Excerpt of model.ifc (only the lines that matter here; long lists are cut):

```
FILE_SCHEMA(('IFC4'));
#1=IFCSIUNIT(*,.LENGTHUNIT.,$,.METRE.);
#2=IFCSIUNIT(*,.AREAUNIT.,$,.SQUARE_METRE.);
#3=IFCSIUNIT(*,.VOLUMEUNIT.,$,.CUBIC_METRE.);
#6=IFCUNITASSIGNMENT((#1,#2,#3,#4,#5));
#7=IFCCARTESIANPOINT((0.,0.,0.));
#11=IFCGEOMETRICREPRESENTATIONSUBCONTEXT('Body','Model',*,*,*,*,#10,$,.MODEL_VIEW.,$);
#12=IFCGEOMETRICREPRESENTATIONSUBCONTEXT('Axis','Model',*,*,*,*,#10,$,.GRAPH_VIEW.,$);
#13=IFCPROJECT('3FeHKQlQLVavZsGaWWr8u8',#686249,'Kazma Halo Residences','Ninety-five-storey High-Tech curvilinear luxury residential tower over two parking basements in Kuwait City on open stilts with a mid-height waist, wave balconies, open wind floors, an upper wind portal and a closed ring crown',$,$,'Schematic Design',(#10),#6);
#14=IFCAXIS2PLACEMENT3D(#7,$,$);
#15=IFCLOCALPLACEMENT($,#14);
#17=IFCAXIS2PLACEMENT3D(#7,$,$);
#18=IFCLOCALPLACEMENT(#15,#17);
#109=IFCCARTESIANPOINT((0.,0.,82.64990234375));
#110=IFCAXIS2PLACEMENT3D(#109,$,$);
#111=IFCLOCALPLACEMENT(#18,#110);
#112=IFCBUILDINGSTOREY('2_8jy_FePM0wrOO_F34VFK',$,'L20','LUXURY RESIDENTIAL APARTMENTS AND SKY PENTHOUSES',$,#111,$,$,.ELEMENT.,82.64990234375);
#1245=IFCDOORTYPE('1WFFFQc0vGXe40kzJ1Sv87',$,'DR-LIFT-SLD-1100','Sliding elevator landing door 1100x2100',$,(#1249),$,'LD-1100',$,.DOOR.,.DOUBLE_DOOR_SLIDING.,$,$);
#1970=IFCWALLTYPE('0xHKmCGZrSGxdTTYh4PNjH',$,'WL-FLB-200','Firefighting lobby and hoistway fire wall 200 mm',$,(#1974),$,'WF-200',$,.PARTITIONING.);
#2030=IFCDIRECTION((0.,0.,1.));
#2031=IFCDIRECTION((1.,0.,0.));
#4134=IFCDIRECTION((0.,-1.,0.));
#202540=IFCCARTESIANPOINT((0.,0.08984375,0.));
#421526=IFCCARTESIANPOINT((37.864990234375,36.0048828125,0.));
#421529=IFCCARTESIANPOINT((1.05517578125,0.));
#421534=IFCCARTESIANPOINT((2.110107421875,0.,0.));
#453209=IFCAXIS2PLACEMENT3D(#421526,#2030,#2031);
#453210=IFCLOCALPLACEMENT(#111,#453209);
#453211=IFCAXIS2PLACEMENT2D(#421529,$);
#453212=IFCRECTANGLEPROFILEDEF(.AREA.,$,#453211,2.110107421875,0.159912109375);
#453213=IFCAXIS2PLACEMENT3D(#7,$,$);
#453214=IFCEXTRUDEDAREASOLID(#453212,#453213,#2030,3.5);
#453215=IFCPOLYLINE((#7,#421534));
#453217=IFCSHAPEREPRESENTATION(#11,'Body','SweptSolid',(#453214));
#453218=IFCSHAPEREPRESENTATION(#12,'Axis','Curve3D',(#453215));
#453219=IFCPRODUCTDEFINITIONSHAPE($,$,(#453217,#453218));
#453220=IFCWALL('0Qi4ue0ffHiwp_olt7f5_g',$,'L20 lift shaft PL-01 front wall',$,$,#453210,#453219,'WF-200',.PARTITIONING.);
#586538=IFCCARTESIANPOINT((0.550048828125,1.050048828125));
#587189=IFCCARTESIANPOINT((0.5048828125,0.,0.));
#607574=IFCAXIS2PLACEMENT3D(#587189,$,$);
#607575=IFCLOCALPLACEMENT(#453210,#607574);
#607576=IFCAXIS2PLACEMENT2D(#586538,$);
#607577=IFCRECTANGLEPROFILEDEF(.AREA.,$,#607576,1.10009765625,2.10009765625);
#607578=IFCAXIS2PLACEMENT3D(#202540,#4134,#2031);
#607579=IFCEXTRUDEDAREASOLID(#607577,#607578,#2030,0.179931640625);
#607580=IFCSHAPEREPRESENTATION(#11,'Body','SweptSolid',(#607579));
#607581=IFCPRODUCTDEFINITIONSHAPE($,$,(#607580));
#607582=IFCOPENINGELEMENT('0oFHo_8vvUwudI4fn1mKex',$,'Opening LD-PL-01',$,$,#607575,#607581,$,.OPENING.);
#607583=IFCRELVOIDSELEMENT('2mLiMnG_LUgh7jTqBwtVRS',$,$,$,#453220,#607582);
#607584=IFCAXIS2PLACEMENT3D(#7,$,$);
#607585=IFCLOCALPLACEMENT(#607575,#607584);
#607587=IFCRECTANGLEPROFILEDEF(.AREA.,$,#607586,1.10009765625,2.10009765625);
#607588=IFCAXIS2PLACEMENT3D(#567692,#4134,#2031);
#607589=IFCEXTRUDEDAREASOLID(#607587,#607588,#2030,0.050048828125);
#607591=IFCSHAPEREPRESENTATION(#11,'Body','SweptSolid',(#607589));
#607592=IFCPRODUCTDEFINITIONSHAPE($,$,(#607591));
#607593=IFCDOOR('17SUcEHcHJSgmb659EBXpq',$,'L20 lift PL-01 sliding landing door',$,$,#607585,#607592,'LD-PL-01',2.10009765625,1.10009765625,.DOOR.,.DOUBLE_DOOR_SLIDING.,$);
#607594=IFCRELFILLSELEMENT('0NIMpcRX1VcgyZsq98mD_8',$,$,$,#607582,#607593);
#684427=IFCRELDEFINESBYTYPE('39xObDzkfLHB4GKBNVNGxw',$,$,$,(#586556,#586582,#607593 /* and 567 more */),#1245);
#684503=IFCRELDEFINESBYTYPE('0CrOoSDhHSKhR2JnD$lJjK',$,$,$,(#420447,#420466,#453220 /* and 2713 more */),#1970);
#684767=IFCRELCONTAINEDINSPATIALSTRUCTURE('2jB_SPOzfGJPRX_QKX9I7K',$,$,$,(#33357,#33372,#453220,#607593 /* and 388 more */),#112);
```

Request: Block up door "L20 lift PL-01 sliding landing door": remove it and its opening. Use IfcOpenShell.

```python
import ifcopenshell
import ifcopenshell.api.feature
import ifcopenshell.api.root
import ifcopenshell.geom
import ifcopenshell.util.shape

model = ifcopenshell.open("model.ifc")
settings = ifcopenshell.geom.settings()


def volume(element):
    """Net volume in cubic metres, openings subtracted."""
    shape = ifcopenshell.geom.create_shape(settings, element)
    return ifcopenshell.util.shape.get_volume(shape.geometry)


door = model.by_guid("17SUcEHcHJSgmb659EBXpq")
opening = door.FillsVoids[0].RelatingOpeningElement
wall = opening.VoidsElements[0].RelatingBuildingElement
before = volume(wall)

ifcopenshell.api.root.remove_product(model, product=door)
ifcopenshell.api.feature.remove_feature(model, feature=opening)

after = volume(wall)

print(f"wall volume {before:.3f} -> {after:.3f} m3")

model.write("model_v2.ifc")
```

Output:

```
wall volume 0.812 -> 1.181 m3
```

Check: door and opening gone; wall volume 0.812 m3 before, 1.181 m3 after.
